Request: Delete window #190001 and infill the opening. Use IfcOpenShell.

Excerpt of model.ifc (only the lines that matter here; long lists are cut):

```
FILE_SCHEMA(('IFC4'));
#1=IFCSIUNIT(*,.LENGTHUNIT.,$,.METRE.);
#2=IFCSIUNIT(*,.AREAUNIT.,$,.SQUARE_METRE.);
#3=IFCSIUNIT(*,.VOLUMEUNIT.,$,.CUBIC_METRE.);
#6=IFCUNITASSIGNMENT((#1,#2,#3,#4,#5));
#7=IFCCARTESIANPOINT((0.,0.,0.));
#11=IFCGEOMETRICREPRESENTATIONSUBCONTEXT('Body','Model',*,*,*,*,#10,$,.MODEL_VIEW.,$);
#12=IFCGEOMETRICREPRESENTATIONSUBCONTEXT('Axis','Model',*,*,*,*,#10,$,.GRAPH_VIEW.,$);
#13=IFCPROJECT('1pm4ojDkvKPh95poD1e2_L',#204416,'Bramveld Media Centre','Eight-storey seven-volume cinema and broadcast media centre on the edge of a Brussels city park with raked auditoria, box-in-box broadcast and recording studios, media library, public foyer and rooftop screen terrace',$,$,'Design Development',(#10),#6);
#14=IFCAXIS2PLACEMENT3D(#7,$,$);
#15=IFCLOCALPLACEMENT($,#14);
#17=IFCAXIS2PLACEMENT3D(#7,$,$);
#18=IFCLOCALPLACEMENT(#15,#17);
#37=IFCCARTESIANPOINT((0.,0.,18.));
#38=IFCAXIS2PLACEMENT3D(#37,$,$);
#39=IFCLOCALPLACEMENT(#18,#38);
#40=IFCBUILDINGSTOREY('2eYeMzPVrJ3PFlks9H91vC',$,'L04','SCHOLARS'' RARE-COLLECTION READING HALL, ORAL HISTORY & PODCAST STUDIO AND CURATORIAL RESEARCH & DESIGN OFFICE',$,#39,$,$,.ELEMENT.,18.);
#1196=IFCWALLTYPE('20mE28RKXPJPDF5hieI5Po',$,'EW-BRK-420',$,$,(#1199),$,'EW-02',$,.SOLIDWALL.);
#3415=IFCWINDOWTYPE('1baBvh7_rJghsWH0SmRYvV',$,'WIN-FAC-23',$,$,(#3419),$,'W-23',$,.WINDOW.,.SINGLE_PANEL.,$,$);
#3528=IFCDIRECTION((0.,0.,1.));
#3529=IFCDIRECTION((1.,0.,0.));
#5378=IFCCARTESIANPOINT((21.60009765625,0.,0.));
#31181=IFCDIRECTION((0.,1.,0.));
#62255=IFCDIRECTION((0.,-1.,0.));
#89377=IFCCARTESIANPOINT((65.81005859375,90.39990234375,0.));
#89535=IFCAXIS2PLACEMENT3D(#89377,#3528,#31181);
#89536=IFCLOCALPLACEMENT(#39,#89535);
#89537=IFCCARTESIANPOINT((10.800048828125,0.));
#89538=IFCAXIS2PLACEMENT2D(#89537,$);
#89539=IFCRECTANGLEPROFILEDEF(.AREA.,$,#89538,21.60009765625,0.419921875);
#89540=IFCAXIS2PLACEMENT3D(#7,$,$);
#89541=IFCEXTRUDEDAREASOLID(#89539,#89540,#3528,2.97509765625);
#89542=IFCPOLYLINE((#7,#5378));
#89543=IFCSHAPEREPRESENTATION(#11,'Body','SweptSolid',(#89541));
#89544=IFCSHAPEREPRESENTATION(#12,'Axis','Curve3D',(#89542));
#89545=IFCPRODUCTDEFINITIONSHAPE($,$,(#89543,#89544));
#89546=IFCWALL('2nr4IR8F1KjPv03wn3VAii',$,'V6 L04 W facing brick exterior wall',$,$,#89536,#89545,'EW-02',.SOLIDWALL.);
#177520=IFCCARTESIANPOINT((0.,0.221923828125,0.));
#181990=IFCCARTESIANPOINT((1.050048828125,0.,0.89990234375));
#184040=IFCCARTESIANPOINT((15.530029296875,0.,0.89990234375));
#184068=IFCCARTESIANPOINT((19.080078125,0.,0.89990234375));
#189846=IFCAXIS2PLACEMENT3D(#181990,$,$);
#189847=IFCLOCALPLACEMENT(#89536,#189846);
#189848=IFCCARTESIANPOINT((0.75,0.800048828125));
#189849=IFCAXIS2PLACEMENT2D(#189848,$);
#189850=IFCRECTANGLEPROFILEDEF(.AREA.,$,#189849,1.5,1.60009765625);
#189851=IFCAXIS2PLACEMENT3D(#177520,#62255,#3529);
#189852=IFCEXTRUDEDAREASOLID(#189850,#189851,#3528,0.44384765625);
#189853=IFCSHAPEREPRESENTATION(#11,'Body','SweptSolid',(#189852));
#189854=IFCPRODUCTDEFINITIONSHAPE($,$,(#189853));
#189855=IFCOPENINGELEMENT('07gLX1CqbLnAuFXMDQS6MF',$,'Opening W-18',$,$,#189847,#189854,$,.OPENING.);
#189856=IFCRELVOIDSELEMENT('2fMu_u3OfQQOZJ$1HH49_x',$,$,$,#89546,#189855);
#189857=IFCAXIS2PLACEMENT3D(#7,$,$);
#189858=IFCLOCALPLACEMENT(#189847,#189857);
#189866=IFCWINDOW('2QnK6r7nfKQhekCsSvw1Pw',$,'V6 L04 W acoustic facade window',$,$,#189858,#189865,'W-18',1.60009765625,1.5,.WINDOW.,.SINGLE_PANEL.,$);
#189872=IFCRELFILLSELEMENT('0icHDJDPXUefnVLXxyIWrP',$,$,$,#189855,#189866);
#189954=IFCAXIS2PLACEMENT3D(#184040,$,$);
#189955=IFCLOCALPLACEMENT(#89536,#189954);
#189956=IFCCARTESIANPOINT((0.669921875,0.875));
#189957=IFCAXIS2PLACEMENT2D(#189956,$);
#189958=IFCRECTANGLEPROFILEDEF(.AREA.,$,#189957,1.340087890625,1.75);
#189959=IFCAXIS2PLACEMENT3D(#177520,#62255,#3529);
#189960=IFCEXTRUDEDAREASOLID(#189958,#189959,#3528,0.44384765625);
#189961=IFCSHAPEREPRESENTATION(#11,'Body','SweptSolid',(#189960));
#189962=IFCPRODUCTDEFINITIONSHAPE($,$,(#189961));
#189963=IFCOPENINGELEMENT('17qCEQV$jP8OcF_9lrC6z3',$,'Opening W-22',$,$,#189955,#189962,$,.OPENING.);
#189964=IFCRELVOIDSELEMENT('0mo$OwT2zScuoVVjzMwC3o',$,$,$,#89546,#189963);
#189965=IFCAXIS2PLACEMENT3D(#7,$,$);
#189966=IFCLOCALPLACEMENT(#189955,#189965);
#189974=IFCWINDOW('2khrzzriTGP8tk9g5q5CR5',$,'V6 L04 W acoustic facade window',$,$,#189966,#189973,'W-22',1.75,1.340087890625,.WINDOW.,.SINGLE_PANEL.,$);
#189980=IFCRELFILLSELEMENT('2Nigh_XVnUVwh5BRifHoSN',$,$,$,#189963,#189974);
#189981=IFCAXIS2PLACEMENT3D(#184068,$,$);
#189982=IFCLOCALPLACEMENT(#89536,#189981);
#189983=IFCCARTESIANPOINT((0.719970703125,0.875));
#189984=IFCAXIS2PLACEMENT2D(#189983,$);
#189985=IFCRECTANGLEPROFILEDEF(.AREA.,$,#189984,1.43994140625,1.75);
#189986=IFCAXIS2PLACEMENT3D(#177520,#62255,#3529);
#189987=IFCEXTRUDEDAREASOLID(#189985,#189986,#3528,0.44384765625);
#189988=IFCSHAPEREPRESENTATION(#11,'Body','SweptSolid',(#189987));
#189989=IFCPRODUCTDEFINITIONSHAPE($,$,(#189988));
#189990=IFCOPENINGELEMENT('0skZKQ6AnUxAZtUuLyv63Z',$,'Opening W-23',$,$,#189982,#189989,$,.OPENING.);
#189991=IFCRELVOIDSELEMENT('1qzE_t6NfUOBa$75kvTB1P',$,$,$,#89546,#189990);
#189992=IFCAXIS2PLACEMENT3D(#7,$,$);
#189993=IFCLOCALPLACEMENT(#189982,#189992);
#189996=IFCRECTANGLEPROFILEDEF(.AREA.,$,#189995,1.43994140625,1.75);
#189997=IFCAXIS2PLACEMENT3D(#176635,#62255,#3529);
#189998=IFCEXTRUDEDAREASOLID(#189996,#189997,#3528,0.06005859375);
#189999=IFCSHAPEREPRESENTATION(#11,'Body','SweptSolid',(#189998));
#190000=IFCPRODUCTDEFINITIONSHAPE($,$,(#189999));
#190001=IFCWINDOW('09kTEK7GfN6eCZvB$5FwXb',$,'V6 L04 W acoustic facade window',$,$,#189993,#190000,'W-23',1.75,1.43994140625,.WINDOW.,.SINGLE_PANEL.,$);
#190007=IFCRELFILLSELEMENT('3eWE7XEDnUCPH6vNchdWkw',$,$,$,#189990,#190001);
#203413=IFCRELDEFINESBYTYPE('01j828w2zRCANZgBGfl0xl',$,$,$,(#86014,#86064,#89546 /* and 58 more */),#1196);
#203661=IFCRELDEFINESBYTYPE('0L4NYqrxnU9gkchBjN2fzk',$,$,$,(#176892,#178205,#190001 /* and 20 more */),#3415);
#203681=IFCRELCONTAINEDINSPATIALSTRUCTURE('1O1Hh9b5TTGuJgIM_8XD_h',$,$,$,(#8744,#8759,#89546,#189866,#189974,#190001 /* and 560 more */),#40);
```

```python
import ifcopenshell
import ifcopenshell.api.feature
import ifcopenshell.api.root
import ifcopenshell.geom
import ifcopenshell.util.shape

model = ifcopenshell.open("model.ifc")
settings = ifcopenshell.geom.settings()


def volume(element):
    """Net volume in cubic metres, openings subtracted."""
    shape = ifcopenshell.geom.create_shape(settings, element)
    return ifcopenshell.util.shape.get_volume(shape.geometry)


window = model.by_guid("09kTEK7GfN6eCZvB$5FwXb")
opening = window.FillsVoids[0].RelatingOpeningElement
wall = opening.VoidsElements[0].RelatingBuildingElement
before = volume(wall)

ifcopenshell.api.root.remove_product(model, product=window)
ifcopenshell.api.feature.remove_feature(model, feature=opening)

after = volume(wall)

print(f"wall volume {before:.3f} -> {after:.3f} m3")

model.write("model_rev.ifc")
```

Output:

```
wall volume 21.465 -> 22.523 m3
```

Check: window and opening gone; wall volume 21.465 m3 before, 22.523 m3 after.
